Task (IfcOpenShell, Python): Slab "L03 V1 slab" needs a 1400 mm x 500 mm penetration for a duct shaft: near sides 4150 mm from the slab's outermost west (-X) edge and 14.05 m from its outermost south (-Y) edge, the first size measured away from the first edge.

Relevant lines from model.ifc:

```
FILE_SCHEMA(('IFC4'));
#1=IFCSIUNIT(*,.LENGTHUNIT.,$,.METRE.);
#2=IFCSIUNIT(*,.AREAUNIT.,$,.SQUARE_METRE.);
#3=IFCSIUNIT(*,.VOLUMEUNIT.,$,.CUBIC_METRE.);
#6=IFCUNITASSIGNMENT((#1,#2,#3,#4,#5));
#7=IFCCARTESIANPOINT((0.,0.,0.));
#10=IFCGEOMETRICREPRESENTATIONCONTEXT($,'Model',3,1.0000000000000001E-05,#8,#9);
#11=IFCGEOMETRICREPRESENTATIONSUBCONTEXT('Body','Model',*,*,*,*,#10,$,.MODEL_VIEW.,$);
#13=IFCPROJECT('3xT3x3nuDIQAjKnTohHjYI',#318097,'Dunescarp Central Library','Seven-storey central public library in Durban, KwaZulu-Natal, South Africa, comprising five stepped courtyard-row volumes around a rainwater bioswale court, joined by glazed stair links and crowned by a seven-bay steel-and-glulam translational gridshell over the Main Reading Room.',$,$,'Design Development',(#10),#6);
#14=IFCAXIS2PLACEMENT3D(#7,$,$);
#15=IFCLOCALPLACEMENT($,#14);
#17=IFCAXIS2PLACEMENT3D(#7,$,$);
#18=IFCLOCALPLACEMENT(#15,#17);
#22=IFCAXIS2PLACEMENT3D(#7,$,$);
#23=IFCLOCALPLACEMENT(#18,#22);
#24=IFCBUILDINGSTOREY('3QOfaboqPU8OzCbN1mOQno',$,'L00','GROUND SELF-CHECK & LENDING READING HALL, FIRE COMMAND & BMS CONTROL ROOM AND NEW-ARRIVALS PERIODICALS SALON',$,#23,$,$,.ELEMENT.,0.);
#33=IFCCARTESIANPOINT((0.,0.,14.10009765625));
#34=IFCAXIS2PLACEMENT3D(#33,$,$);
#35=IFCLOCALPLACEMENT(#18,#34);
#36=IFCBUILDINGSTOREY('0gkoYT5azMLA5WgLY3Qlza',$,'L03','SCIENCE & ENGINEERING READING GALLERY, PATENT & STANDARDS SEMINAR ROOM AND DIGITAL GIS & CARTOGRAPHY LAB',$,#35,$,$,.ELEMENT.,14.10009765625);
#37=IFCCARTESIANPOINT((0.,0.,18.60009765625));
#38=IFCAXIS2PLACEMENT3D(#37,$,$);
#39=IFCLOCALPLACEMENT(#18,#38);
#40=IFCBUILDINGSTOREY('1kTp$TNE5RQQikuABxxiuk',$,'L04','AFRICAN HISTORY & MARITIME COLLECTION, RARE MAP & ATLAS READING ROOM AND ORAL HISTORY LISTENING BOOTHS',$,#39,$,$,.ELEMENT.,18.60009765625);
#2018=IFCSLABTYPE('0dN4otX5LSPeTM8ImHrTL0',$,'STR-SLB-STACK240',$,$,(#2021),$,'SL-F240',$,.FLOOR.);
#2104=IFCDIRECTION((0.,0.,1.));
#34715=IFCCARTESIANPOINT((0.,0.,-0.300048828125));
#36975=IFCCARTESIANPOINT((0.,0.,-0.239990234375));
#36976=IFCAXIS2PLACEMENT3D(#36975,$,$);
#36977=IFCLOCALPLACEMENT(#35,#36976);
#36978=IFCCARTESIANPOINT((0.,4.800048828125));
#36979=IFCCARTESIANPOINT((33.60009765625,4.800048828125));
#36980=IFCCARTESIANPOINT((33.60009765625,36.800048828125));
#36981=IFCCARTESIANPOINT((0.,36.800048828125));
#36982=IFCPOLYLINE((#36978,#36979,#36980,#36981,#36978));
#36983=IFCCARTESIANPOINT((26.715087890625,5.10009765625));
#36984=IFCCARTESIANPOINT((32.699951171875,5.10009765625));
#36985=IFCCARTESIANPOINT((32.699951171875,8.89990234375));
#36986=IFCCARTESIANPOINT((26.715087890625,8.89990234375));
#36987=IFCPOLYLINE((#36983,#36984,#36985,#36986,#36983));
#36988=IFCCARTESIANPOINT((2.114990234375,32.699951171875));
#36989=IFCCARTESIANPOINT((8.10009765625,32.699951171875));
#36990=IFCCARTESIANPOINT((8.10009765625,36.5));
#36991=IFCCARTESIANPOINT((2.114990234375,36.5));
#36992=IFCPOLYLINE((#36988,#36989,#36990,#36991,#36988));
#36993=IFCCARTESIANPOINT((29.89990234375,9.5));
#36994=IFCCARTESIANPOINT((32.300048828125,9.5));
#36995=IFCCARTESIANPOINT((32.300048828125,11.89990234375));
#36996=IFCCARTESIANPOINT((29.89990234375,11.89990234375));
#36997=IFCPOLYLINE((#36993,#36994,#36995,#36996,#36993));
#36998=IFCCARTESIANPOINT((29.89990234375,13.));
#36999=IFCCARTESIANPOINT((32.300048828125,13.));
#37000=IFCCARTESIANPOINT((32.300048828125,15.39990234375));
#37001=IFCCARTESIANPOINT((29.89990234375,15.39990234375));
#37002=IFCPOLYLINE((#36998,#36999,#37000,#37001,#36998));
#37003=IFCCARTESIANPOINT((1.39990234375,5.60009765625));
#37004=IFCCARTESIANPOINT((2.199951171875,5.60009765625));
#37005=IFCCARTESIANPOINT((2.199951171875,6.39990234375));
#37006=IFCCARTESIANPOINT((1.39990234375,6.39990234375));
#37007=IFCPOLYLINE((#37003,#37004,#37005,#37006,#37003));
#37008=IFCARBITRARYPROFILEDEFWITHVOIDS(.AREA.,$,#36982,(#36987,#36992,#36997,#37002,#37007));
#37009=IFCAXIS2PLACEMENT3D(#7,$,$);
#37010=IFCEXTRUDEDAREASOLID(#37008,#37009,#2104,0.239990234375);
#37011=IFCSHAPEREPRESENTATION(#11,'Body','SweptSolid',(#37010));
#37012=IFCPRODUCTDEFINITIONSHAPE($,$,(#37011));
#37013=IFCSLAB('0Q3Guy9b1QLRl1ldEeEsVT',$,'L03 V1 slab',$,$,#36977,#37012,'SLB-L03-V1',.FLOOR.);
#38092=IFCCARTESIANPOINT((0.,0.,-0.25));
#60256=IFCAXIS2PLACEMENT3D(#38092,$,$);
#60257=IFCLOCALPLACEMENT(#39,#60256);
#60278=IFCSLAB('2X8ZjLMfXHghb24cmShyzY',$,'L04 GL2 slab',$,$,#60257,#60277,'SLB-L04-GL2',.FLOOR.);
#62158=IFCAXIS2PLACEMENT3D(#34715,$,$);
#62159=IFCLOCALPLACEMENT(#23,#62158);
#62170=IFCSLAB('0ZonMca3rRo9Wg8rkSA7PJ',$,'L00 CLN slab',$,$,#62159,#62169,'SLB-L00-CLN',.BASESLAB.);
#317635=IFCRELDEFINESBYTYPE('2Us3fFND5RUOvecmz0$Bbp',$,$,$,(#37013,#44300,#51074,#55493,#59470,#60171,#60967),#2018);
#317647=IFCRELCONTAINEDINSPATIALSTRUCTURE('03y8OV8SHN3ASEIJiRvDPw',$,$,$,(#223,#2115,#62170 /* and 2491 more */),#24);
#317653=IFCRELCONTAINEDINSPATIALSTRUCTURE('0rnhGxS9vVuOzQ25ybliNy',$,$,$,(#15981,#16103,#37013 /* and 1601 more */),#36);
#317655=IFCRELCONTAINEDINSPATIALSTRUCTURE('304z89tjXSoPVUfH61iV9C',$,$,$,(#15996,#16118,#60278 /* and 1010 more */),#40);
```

```python
import numpy as np
import ifcopenshell
import ifcopenshell.api.feature
import ifcopenshell.api.geometry
import ifcopenshell.api.root
import ifcopenshell.geom
import ifcopenshell.util.placement
import ifcopenshell.util.representation
import ifcopenshell.util.shape
import ifcopenshell.util.unit

model = ifcopenshell.open("model.ifc")
unit_scale = ifcopenshell.util.unit.calculate_unit_scale(model)
settings = ifcopenshell.geom.settings()


def volume(element):
    """Net volume in cubic metres, openings subtracted."""
    shape = ifcopenshell.geom.create_shape(settings, element)
    return ifcopenshell.util.shape.get_volume(shape.geometry)


slab = model.by_guid("0Q3Guy9b1QLRl1ldEeEsVT")
before = volume(slab)

# Extent in the slab's own axes, in metres. The edges named are its -X and -Y sides.
slab_shape = ifcopenshell.geom.create_shape(settings, slab)
vertices = ifcopenshell.util.shape.get_vertices(slab_shape.geometry)
x_min, y_min, bottom = vertices.min(axis=0)
top = vertices[:, 2].max()

opening = ifcopenshell.api.root.create_entity(model, ifc_class="IfcOpeningElement", name="Duct shaft opening", predefined_type="OPENING")
context = ifcopenshell.util.representation.get_context(model, "Model", "Body", "MODEL_VIEW")
width, depth = 1.4, 0.5
outline = [(0.0, 0.0), (width, 0.0), (width, depth), (0.0, depth), (0.0, 0.0)]
# Overshoot both faces by 50 mm so the cut is clean.
shape = ifcopenshell.api.geometry.add_slab_representation(
    model, context=context, depth=top - bottom + 0.1, polyline=outline
)
ifcopenshell.api.geometry.assign_representation(model, product=opening, representation=shape)

matrix = ifcopenshell.util.placement.get_local_placement(slab.ObjectPlacement)
matrix[:, 3] = matrix @ np.append(np.array([x_min + 4.15, y_min + 14.05, bottom - 0.05]) / unit_scale, 1.0)
ifcopenshell.api.geometry.edit_object_placement(model, product=opening, matrix=matrix, is_si=False)
ifcopenshell.api.feature.add_feature(model, feature=opening, element=slab)

after = volume(slab)

print(f"slab volume {before:.3f} -> {after:.3f} m3")

model.write("model-out.ifc")
```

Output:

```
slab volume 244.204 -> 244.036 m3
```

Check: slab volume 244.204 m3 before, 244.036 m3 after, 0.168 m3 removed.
